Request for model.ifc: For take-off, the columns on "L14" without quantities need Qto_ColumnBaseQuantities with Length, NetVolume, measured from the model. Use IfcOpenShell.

First a look at what the model holds.

```python
import ifcopenshell
import ifcopenshell.util.element
import ifcopenshell.util.unit

model = ifcopenshell.open("model.ifc")
print(model.schema)
for unit_type in ("LENGTHUNIT", "AREAUNIT", "VOLUMEUNIT"):
    print(unit_type, ifcopenshell.util.unit.calculate_unit_scale(model, unit_type))
storey = next(s for s in model.by_type("IfcBuildingStorey") if s.Name == "L14")
columns = [e for e in ifcopenshell.util.element.get_decomposition(storey) if e.is_a("IfcColumn")]
for e in sorted(columns, key=lambda e: e.id()):
    print(e.id(), e.is_a(), e.Name, list(ifcopenshell.util.element.get_psets(e, qtos_only=True)), sep=" | ")
```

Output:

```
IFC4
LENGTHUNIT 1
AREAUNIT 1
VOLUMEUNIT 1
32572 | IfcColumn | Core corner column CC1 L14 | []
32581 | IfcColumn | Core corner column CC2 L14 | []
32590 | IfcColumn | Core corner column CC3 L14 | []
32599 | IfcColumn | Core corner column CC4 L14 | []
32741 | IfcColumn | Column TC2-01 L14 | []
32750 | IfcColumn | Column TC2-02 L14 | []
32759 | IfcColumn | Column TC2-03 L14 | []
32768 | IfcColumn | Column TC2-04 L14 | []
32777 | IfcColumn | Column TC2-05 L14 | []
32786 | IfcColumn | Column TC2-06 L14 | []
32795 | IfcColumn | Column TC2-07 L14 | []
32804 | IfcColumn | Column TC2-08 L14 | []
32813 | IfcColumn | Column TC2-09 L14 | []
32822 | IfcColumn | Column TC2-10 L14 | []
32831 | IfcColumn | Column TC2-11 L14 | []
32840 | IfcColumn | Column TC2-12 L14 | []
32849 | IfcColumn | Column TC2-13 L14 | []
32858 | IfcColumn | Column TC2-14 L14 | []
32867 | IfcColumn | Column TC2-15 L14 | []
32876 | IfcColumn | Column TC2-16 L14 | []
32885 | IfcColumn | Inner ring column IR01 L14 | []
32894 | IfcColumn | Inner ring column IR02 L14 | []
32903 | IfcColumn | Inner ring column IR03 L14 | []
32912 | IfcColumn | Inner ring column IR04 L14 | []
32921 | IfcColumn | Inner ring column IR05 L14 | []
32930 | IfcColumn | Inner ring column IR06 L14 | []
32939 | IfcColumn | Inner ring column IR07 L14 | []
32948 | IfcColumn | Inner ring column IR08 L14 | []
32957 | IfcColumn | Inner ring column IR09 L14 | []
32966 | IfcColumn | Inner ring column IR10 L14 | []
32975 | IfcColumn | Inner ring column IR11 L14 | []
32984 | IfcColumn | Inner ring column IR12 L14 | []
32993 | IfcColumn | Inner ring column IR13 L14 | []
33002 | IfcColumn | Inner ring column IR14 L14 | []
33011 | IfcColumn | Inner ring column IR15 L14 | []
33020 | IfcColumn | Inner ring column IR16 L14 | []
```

```python
import ifcopenshell
import ifcopenshell.api.pset
import ifcopenshell.geom
import ifcopenshell.util.element
import ifcopenshell.util.shape
import ifcopenshell.util.unit

model = ifcopenshell.open("model.ifc")
unit_scale = ifcopenshell.util.unit.calculate_unit_scale(model)
volume_scale = ifcopenshell.util.unit.calculate_unit_scale(model, "VOLUMEUNIT")
settings = ifcopenshell.geom.settings()

storey = next(s for s in model.by_type("IfcBuildingStorey") if s.Name == "L14")
columns = [e for e in ifcopenshell.util.element.get_decomposition(storey) if e.is_a("IfcColumn")]

for e in sorted(columns, key=lambda e: e.id()):
    if ifcopenshell.util.element.get_psets(e, qtos_only=True, should_inherit=False):
        continue
    # Geometry comes back in metres, in the element's own axes.
    shape = ifcopenshell.geom.create_shape(settings, e)
    values = {
        "Length": ifcopenshell.util.shape.get_z(shape.geometry) / unit_scale,
        "NetVolume": ifcopenshell.util.shape.get_volume(shape.geometry) / volume_scale,
    }
    qto = ifcopenshell.api.pset.add_qto(model, product=e, name="Qto_ColumnBaseQuantities")
    ifcopenshell.api.pset.edit_qto(model, qto=qto, properties=values)
    print(e.id(), {k: round(v, 3) for k, v in values.items()})

model.write("model_updated.ifc")
```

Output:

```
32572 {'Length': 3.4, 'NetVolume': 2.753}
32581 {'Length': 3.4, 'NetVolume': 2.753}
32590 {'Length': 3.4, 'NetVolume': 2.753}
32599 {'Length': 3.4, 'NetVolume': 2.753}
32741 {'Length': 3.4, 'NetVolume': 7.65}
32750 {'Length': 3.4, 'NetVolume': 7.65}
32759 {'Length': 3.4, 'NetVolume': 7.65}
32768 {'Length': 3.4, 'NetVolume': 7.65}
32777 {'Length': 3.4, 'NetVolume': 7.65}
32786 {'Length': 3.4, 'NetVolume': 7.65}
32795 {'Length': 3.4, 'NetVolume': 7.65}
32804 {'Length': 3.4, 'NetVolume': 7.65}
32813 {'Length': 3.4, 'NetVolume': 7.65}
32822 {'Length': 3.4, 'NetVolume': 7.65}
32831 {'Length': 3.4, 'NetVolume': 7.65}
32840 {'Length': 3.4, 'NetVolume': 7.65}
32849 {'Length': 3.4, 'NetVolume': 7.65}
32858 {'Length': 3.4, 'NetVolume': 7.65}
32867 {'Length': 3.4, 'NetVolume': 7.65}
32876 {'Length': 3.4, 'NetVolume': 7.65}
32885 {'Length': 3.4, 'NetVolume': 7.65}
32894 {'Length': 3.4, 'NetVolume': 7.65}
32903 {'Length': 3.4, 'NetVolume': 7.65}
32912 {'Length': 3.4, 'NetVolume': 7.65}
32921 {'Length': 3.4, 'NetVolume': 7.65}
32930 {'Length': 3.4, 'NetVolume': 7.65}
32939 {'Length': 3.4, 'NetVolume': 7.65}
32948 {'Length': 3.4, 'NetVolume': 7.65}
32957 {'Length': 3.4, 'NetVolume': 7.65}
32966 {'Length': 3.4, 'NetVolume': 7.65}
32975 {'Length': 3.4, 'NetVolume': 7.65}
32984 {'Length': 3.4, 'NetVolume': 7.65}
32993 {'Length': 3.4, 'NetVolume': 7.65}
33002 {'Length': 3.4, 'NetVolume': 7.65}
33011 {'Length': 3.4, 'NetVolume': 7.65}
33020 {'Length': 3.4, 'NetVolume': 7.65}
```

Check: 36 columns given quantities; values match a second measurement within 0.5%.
